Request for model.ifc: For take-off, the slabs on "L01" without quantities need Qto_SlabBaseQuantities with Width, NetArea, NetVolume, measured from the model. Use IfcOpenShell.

First a look at what the model holds.

```python
import ifcopenshell
import ifcopenshell.util.element
import ifcopenshell.util.unit

model = ifcopenshell.open("model.ifc")
print(model.schema)
for unit_type in ("LENGTHUNIT", "AREAUNIT", "VOLUMEUNIT"):
    print(unit_type, ifcopenshell.util.unit.calculate_unit_scale(model, unit_type))
storey = next(s for s in model.by_type("IfcBuildingStorey") if s.Name == "L01")
slabs = [e for e in ifcopenshell.util.element.get_decomposition(storey) if e.is_a("IfcSlab")]
for e in sorted(slabs, key=lambda e: e.id()):
    print(e.id(), e.is_a(), e.Name, list(ifcopenshell.util.element.get_psets(e, qtos_only=True)), sep=" | ")
```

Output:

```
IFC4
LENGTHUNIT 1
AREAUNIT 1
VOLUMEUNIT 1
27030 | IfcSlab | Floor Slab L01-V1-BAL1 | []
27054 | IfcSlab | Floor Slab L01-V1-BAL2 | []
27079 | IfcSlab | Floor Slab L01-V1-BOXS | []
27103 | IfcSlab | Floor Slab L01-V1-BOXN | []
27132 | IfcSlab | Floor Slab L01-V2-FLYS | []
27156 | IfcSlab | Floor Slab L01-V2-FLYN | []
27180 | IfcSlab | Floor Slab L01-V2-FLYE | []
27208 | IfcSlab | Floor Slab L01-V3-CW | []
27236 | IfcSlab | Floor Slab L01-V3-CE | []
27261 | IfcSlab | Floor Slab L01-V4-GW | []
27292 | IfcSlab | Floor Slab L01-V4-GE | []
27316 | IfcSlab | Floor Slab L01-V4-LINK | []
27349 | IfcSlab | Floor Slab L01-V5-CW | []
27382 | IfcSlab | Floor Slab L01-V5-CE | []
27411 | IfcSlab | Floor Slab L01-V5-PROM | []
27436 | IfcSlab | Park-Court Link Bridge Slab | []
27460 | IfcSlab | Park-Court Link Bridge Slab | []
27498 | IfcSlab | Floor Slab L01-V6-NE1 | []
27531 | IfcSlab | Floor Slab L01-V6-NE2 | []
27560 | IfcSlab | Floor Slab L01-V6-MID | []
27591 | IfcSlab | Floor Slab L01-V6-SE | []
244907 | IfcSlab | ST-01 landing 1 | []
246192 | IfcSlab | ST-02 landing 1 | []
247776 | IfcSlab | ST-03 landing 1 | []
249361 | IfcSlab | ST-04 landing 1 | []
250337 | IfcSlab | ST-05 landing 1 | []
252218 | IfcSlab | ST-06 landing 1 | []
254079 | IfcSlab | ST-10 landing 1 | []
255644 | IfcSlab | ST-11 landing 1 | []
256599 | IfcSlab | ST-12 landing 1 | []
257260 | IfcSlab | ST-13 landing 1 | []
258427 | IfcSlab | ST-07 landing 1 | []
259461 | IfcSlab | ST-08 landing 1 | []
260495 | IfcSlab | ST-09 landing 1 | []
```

```python
import ifcopenshell
import ifcopenshell.api.pset
import ifcopenshell.geom
import ifcopenshell.util.element
import ifcopenshell.util.shape
import ifcopenshell.util.unit

model = ifcopenshell.open("model.ifc")
unit_scale = ifcopenshell.util.unit.calculate_unit_scale(model)
area_scale = ifcopenshell.util.unit.calculate_unit_scale(model, "AREAUNIT")
volume_scale = ifcopenshell.util.unit.calculate_unit_scale(model, "VOLUMEUNIT")
settings = ifcopenshell.geom.settings()

storey = next(s for s in model.by_type("IfcBuildingStorey") if s.Name == "L01")
slabs = [e for e in ifcopenshell.util.element.get_decomposition(storey) if e.is_a("IfcSlab")]

for e in sorted(slabs, key=lambda e: e.id()):
    if ifcopenshell.util.element.get_psets(e, qtos_only=True, should_inherit=False):
        continue
    # Geometry comes back in metres, in the element's own axes.
    shape = ifcopenshell.geom.create_shape(settings, e)
    values = {
        "Width": ifcopenshell.util.shape.get_z(shape.geometry) / unit_scale,
        "NetArea": ifcopenshell.util.shape.get_footprint_area(shape.geometry) / area_scale,
        "NetVolume": ifcopenshell.util.shape.get_volume(shape.geometry) / volume_scale,
    }
    qto = ifcopenshell.api.pset.add_qto(model, product=e, name="Qto_SlabBaseQuantities")
    ifcopenshell.api.pset.edit_qto(model, qto=qto, properties=values)
    print(e.id(), {k: round(v, 3) for k, v in values.items()})

model.write("model_edited.ifc")
```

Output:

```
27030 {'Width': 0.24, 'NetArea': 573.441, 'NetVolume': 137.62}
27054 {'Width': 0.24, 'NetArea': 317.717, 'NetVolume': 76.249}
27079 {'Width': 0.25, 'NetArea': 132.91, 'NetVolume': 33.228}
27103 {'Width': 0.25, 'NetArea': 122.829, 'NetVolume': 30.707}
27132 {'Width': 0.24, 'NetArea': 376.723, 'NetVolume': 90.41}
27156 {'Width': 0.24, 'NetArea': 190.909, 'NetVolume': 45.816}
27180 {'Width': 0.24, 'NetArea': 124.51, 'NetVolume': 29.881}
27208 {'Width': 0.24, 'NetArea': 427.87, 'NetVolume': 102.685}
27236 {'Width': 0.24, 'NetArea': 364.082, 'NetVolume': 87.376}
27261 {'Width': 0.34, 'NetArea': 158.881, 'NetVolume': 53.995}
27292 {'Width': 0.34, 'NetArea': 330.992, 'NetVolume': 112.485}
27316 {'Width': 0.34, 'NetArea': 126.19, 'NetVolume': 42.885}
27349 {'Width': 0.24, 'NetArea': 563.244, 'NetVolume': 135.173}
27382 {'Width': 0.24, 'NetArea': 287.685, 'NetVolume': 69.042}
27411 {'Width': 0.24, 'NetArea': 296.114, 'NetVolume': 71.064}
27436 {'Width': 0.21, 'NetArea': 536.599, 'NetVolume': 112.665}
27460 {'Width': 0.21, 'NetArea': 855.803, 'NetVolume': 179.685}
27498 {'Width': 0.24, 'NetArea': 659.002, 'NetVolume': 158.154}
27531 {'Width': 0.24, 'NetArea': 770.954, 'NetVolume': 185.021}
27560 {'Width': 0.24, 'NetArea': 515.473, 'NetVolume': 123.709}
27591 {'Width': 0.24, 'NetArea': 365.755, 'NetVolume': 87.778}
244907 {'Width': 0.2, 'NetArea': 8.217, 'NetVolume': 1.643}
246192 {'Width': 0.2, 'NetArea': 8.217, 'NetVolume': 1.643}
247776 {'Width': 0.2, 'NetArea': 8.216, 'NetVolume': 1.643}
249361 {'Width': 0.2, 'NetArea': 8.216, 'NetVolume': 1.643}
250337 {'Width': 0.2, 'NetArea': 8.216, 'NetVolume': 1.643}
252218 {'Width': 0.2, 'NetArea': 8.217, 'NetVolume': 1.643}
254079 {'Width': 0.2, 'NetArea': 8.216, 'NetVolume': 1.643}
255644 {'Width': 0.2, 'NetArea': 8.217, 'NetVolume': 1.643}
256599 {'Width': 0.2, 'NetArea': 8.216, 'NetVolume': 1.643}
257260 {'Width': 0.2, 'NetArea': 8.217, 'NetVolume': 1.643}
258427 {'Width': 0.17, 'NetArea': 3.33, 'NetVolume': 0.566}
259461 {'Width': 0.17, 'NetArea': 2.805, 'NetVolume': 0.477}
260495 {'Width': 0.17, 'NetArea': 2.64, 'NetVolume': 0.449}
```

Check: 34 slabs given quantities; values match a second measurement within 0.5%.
